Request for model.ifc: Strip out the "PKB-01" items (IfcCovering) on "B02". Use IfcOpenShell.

First a look at what the model holds.

```python
import ifcopenshell
import ifcopenshell.util.element

model = ifcopenshell.open("model.ifc")
print(model.schema)
storey = next(s for s in model.by_type("IfcBuildingStorey") if s.Name == "B02")
coverings = [e for e in ifcopenshell.util.element.get_decomposition(storey) if e.is_a("IfcCovering")]
seen = {}
for e in coverings:
    element_type = ifcopenshell.util.element.get_type(e)
    name = element_type.Name if element_type not in (None, e) else None
    seen[name] = seen.get(name, 0) + 1
for name, count in sorted(seen.items(), key=str):
    print(count, "x", name)
```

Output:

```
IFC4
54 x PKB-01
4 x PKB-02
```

```python
import ifcopenshell
import ifcopenshell.api.root
import ifcopenshell.util.element

model = ifcopenshell.open("model.ifc")

storey = next(s for s in model.by_type("IfcBuildingStorey") if s.Name == "B02")
coverings = [e for e in ifcopenshell.util.element.get_decomposition(storey) if e.is_a("IfcCovering")]
targets = [e for e in coverings if (t := ifcopenshell.util.element.get_type(e)) not in (None, e) and t.Name == "PKB-01"]

for e in targets:
    ifcopenshell.api.root.remove_product(model, product=e)
print(len(targets), "removed")

model.write("model-out.ifc")
```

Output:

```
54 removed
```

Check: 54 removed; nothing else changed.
